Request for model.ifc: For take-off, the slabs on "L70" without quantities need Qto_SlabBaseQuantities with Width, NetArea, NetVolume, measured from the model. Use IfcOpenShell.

First a look at what the model holds.

```python
import ifcopenshell
import ifcopenshell.util.element
import ifcopenshell.util.unit

model = ifcopenshell.open("model.ifc")
print(model.schema)
for unit_type in ("LENGTHUNIT", "AREAUNIT", "VOLUMEUNIT"):
    print(unit_type, ifcopenshell.util.unit.calculate_unit_scale(model, unit_type))
storey = next(s for s in model.by_type("IfcBuildingStorey") if s.Name == "L70")
slabs = [e for e in ifcopenshell.util.element.get_decomposition(storey) if e.is_a("IfcSlab")]
for e in sorted(slabs, key=lambda e: e.id()):
    print(e.id(), e.is_a(), e.Name, list(ifcopenshell.util.element.get_psets(e, qtos_only=True)), sep=" | ")
```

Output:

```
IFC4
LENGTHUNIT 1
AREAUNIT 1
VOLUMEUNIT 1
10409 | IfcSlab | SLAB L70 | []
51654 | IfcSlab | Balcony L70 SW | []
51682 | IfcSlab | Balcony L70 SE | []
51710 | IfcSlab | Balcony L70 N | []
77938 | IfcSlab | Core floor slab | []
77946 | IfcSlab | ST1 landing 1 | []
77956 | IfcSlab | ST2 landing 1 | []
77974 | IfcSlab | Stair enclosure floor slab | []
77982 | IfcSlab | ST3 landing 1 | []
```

```python
import ifcopenshell
import ifcopenshell.api.pset
import ifcopenshell.geom
import ifcopenshell.util.element
import ifcopenshell.util.shape
import ifcopenshell.util.unit

model = ifcopenshell.open("model.ifc")
unit_scale = ifcopenshell.util.unit.calculate_unit_scale(model)
area_scale = ifcopenshell.util.unit.calculate_unit_scale(model, "AREAUNIT")
volume_scale = ifcopenshell.util.unit.calculate_unit_scale(model, "VOLUMEUNIT")
settings = ifcopenshell.geom.settings()

storey = next(s for s in model.by_type("IfcBuildingStorey") if s.Name == "L70")
slabs = [e for e in ifcopenshell.util.element.get_decomposition(storey) if e.is_a("IfcSlab")]

for e in sorted(slabs, key=lambda e: e.id()):
    if ifcopenshell.util.element.get_psets(e, qtos_only=True, should_inherit=False):
        continue
    # Geometry comes back in metres, in the element's own axes.
    shape = ifcopenshell.geom.create_shape(settings, e)
    values = {
        "Width": ifcopenshell.util.shape.get_z(shape.geometry) / unit_scale,
        "NetArea": ifcopenshell.util.shape.get_footprint_area(shape.geometry) / area_scale,
        "NetVolume": ifcopenshell.util.shape.get_volume(shape.geometry) / volume_scale,
    }
    qto = ifcopenshell.api.pset.add_qto(model, product=e, name="Qto_SlabBaseQuantities")
    ifcopenshell.api.pset.edit_qto(model, qto=qto, properties=values)
    print(e.id(), {k: round(v, 3) for k, v in values.items()})

model.write("model_updated.ifc")
```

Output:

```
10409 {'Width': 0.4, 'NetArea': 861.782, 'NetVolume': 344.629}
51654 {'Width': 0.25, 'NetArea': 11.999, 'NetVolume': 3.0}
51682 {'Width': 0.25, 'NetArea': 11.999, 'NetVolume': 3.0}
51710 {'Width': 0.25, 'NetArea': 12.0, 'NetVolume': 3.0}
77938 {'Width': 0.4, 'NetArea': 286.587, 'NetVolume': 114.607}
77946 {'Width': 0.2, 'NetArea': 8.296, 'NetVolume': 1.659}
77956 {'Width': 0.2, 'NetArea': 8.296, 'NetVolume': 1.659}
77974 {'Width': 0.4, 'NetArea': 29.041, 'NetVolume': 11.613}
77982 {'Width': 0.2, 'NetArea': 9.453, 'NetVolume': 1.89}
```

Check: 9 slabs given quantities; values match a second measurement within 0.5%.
